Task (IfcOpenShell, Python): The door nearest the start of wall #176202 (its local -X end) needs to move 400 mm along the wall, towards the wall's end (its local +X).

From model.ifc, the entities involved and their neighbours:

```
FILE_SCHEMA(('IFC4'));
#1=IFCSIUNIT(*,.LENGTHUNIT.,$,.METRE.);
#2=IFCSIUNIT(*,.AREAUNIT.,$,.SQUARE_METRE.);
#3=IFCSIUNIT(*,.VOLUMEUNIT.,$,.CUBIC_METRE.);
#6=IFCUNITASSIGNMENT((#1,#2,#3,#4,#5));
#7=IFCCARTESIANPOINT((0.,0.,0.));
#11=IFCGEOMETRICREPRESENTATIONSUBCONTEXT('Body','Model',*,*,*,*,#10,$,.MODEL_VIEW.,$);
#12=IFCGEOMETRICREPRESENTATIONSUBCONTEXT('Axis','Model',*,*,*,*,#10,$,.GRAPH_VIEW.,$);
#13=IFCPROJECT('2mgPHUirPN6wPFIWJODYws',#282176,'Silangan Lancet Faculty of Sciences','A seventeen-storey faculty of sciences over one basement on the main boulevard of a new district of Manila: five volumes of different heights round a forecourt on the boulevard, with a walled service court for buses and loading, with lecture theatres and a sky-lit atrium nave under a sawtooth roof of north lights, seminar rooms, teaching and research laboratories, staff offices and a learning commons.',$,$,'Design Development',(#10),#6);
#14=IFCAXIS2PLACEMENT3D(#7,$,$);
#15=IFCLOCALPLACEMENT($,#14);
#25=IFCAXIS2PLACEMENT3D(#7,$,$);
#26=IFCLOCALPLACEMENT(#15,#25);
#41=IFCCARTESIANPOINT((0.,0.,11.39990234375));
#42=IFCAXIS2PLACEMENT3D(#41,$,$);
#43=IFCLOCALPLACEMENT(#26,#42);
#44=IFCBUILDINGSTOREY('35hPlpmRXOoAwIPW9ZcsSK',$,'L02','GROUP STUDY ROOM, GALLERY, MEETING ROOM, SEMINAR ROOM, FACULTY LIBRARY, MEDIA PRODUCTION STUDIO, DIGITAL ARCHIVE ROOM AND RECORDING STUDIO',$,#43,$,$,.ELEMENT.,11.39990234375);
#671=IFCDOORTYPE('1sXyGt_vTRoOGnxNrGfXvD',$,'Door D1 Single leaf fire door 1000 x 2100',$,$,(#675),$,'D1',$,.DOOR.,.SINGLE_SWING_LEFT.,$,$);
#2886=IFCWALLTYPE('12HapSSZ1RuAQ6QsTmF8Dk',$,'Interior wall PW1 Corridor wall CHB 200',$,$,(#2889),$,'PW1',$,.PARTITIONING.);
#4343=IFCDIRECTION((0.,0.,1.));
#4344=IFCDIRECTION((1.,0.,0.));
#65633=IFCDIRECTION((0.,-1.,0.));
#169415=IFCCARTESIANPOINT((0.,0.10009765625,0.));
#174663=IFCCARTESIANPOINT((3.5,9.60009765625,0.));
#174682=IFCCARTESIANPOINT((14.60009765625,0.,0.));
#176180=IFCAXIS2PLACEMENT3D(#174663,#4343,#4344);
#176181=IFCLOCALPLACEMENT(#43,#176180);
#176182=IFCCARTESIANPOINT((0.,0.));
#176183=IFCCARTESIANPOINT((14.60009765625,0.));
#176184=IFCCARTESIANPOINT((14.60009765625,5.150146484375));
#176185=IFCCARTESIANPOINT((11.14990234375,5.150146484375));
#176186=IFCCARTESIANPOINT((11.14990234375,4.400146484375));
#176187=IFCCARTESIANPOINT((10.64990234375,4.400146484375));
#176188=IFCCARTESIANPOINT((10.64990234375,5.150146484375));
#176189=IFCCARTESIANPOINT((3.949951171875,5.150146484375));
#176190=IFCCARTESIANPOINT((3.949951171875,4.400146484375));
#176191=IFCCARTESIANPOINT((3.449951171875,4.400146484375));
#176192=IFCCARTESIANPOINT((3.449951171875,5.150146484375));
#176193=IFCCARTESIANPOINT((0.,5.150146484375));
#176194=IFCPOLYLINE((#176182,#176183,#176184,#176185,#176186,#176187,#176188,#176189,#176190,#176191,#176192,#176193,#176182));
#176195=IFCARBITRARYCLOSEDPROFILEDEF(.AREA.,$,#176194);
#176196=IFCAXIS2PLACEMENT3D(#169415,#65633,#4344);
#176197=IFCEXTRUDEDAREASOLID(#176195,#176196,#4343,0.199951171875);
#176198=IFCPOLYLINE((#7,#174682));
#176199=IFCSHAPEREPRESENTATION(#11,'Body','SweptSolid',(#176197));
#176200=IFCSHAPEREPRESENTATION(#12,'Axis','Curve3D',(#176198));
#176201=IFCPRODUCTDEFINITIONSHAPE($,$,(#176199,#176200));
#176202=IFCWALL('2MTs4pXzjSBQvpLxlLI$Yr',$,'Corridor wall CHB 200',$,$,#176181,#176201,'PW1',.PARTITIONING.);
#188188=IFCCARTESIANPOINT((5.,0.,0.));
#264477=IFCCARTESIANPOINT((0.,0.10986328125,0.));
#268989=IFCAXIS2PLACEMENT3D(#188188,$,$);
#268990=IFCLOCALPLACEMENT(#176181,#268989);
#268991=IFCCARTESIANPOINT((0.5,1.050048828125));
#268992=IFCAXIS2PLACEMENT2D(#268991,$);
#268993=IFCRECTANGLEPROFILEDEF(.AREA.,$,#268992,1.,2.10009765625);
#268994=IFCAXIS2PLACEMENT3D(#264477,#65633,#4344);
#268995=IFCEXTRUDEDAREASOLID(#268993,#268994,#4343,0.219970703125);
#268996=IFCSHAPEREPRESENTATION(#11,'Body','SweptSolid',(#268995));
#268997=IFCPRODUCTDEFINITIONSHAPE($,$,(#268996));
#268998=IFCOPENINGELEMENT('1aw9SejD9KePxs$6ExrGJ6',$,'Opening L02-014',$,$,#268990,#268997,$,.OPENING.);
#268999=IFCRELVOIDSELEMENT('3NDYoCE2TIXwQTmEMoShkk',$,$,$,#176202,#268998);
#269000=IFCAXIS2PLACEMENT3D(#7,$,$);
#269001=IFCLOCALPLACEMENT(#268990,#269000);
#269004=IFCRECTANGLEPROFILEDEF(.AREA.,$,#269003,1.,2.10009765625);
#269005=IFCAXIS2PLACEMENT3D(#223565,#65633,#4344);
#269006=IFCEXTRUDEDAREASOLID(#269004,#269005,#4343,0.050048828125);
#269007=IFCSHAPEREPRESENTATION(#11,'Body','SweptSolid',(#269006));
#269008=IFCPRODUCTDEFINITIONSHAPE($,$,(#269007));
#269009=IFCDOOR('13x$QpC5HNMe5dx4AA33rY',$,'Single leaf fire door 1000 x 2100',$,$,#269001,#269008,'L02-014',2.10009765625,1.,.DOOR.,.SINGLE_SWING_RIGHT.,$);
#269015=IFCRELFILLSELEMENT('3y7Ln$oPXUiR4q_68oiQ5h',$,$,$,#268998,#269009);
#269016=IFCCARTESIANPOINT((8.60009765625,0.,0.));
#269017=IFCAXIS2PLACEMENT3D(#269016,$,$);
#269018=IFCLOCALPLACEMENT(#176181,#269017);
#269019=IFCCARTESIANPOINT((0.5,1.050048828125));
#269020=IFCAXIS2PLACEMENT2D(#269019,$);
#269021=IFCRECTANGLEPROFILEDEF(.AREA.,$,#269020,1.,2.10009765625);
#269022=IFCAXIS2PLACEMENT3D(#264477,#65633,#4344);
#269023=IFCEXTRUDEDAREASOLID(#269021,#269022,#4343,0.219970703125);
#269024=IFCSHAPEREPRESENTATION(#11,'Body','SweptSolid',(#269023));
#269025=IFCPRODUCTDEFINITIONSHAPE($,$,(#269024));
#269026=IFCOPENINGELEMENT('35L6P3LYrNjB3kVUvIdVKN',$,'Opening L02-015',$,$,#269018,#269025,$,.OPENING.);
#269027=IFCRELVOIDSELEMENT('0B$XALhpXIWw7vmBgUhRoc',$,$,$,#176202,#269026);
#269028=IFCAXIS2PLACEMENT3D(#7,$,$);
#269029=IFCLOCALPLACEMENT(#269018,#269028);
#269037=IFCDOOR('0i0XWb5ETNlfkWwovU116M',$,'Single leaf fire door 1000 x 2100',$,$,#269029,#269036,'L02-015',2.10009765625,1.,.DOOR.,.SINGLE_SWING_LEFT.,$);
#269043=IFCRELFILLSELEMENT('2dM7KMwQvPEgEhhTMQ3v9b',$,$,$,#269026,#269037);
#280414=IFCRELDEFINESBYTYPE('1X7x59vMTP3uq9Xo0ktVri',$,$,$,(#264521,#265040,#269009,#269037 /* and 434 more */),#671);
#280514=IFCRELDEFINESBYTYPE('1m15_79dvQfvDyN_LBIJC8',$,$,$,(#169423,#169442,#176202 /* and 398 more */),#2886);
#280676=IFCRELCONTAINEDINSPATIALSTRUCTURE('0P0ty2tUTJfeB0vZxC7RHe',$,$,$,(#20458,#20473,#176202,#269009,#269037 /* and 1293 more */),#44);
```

```python
import ifcopenshell
import ifcopenshell.api.geometry
import ifcopenshell.util.placement

model = ifcopenshell.open("model.ifc")

door = model.by_guid("13x$QpC5HNMe5dx4AA33rY")
opening = door.FillsVoids[0].RelatingOpeningElement
wall = opening.VoidsElements[0].RelatingBuildingElement

wall_matrix = ifcopenshell.util.placement.get_local_placement(wall.ObjectPlacement)
shift = wall_matrix[:3, 0] * 0.4
before = ifcopenshell.util.placement.get_local_placement(door.ObjectPlacement)[:3, 3].copy()

# The door is placed relative to its opening, so it follows when the opening moves.
matrix = ifcopenshell.util.placement.get_local_placement(opening.ObjectPlacement)
matrix[:3, 3] += shift
ifcopenshell.api.geometry.edit_object_placement(
    model, product=opening, matrix=matrix, is_si=False, should_transform_children=True
)

after = ifcopenshell.util.placement.get_local_placement(door.ObjectPlacement)[:3, 3]
print("door moved by", (after - before).round(3) + 0.0)

model.write("model_v2.ifc")
```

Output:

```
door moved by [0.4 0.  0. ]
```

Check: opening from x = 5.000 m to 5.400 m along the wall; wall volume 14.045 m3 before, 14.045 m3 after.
